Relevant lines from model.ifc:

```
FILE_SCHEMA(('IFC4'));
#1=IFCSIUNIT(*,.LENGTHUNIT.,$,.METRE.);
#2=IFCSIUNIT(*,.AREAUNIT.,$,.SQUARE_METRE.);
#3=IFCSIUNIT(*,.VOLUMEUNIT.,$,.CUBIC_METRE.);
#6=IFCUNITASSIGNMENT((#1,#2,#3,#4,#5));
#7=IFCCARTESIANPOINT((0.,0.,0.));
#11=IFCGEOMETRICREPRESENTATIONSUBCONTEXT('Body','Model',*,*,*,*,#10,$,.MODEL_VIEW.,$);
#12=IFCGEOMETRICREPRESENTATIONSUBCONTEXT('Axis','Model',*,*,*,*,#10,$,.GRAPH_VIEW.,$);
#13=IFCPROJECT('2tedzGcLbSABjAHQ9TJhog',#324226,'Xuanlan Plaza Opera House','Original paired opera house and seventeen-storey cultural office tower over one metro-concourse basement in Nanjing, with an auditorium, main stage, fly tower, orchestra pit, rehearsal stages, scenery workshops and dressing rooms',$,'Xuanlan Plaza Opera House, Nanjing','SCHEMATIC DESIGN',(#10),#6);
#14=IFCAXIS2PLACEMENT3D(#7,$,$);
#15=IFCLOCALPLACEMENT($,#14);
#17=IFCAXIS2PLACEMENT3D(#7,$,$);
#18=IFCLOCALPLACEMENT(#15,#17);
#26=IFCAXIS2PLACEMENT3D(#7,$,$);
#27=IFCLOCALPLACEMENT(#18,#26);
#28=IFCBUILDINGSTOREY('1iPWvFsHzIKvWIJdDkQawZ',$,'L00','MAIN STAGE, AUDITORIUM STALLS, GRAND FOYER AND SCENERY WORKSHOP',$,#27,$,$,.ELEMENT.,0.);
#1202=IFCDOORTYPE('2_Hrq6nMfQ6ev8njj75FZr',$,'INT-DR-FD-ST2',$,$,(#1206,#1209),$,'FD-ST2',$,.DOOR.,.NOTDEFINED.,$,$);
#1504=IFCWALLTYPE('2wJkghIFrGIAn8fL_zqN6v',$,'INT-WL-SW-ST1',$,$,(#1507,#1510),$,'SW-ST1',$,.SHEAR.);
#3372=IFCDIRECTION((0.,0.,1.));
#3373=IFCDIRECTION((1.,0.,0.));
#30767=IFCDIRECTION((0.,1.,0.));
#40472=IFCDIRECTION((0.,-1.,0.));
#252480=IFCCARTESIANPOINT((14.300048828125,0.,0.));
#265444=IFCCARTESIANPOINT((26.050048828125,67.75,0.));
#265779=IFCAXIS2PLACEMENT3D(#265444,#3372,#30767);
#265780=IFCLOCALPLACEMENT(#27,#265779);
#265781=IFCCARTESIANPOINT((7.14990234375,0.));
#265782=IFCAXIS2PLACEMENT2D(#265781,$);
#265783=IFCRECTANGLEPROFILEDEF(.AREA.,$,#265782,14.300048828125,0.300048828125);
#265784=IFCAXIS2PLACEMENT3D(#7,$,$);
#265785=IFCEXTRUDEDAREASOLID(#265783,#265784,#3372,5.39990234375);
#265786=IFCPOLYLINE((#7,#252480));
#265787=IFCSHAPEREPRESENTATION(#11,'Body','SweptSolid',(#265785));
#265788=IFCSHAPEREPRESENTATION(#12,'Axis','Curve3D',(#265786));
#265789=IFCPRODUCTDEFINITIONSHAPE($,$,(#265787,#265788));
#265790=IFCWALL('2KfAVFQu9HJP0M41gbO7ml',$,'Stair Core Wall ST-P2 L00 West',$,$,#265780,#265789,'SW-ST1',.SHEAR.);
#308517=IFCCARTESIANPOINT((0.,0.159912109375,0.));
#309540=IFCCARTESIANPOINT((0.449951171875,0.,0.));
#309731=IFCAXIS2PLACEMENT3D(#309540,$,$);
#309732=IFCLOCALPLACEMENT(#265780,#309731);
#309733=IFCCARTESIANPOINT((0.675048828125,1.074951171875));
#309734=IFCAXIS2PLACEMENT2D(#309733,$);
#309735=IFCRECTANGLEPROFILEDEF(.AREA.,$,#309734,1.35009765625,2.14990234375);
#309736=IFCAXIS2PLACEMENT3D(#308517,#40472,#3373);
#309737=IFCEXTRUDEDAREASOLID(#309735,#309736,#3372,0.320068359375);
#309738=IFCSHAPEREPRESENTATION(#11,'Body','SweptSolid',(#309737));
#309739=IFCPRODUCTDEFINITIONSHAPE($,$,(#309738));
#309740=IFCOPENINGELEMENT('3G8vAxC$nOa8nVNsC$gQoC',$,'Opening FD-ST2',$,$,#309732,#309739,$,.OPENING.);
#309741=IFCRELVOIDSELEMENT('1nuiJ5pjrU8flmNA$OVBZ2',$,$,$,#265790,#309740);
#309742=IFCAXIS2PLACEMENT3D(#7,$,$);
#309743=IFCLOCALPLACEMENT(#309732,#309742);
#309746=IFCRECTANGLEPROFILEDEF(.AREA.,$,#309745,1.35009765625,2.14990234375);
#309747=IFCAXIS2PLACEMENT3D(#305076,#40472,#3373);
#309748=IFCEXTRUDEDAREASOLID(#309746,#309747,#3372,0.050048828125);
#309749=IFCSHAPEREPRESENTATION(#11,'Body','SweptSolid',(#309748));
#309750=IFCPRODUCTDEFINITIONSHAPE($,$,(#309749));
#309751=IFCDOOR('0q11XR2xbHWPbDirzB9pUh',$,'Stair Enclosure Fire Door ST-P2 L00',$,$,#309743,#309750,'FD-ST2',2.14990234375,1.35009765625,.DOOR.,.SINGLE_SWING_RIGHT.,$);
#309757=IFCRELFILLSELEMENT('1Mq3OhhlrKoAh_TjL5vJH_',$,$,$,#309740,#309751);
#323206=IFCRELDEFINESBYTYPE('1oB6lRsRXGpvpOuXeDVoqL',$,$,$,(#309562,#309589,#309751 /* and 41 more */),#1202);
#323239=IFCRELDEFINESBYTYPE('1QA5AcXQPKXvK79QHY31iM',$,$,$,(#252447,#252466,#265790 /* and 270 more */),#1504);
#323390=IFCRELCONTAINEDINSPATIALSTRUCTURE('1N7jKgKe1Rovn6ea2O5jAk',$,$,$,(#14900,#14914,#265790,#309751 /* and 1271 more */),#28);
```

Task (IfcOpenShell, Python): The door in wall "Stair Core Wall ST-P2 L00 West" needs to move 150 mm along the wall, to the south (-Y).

```python
import ifcopenshell
import ifcopenshell.api.geometry
import ifcopenshell.util.placement

model = ifcopenshell.open("model.ifc")

door = model.by_guid("0q11XR2xbHWPbDirzB9pUh")
opening = door.FillsVoids[0].RelatingOpeningElement
wall = opening.VoidsElements[0].RelatingBuildingElement

wall_matrix = ifcopenshell.util.placement.get_local_placement(wall.ObjectPlacement)
shift = wall_matrix[:3, 0] * -0.15
before = ifcopenshell.util.placement.get_local_placement(door.ObjectPlacement)[:3, 3].copy()

# The door is placed relative to its opening, so it follows when the opening moves.
matrix = ifcopenshell.util.placement.get_local_placement(opening.ObjectPlacement)
matrix[:3, 3] += shift
ifcopenshell.api.geometry.edit_object_placement(
    model, product=opening, matrix=matrix, is_si=False, should_transform_children=True
)

after = ifcopenshell.util.placement.get_local_placement(door.ObjectPlacement)[:3, 3]
print("door moved by", (after - before).round(3) + 0.0)

model.write("model_updated.ifc")
```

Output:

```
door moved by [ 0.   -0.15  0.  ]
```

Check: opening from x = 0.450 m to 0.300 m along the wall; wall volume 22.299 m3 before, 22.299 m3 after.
